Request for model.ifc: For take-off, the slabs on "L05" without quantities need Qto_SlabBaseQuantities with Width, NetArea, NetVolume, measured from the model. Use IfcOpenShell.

First a look at what the model holds.

```python
import ifcopenshell
import ifcopenshell.util.element
import ifcopenshell.util.unit

model = ifcopenshell.open("model.ifc")
print(model.schema)
for unit_type in ("LENGTHUNIT", "AREAUNIT", "VOLUMEUNIT"):
    print(unit_type, ifcopenshell.util.unit.calculate_unit_scale(model, unit_type))
storey = next(s for s in model.by_type("IfcBuildingStorey") if s.Name == "L05")
slabs = [e for e in ifcopenshell.util.element.get_decomposition(storey) if e.is_a("IfcSlab")]
for e in sorted(slabs, key=lambda e: e.id()):
    print(e.id(), e.is_a(), e.Name, list(ifcopenshell.util.element.get_psets(e, qtos_only=True)), sep=" | ")
```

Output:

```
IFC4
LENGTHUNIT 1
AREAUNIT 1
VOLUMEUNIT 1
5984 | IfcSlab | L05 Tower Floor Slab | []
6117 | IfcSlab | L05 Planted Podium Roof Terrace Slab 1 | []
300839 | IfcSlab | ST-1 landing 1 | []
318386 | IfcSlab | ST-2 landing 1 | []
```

```python
import ifcopenshell
import ifcopenshell.api.pset
import ifcopenshell.geom
import ifcopenshell.util.element
import ifcopenshell.util.shape
import ifcopenshell.util.unit

model = ifcopenshell.open("model.ifc")
unit_scale = ifcopenshell.util.unit.calculate_unit_scale(model)
area_scale = ifcopenshell.util.unit.calculate_unit_scale(model, "AREAUNIT")
volume_scale = ifcopenshell.util.unit.calculate_unit_scale(model, "VOLUMEUNIT")
settings = ifcopenshell.geom.settings()

storey = next(s for s in model.by_type("IfcBuildingStorey") if s.Name == "L05")
slabs = [e for e in ifcopenshell.util.element.get_decomposition(storey) if e.is_a("IfcSlab")]

for e in sorted(slabs, key=lambda e: e.id()):
    if ifcopenshell.util.element.get_psets(e, qtos_only=True, should_inherit=False):
        continue
    # Geometry comes back in metres, in the element's own axes.
    shape = ifcopenshell.geom.create_shape(settings, e)
    values = {
        "Width": ifcopenshell.util.shape.get_z(shape.geometry) / unit_scale,
        "NetArea": ifcopenshell.util.shape.get_footprint_area(shape.geometry) / area_scale,
        "NetVolume": ifcopenshell.util.shape.get_volume(shape.geometry) / volume_scale,
    }
    qto = ifcopenshell.api.pset.add_qto(model, product=e, name="Qto_SlabBaseQuantities")
    ifcopenshell.api.pset.edit_qto(model, qto=qto, properties=values)
    print(e.id(), {k: round(v, 3) for k, v in values.items()})

model.write("model_updated.ifc")
```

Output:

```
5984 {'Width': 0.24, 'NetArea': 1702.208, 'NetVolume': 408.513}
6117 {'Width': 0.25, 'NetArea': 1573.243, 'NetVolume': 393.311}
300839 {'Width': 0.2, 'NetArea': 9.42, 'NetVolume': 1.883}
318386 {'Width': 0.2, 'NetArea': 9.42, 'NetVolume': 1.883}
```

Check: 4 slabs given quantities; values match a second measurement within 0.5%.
